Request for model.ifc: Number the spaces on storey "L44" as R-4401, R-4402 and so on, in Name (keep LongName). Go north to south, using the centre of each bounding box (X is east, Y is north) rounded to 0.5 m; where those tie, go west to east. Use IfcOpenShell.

First a look at what the model holds.

```python
import ifcopenshell
import ifcopenshell.util.element
import ifcopenshell.util.placement

model = ifcopenshell.open("model.ifc")
print(model.schema)
storey = next(s for s in model.by_type("IfcBuildingStorey") if s.Name == "L44")
spaces = [e for e in ifcopenshell.util.element.get_decomposition(storey) if e.is_a("IfcSpace")]
for e in sorted(spaces, key=lambda e: e.id()):
    origin = ifcopenshell.util.placement.get_local_placement(e.ObjectPlacement)[:3, 3]
    print(e.id(), e.Name, e.LongName, origin.round(2) + 0.0, sep=" | ")
```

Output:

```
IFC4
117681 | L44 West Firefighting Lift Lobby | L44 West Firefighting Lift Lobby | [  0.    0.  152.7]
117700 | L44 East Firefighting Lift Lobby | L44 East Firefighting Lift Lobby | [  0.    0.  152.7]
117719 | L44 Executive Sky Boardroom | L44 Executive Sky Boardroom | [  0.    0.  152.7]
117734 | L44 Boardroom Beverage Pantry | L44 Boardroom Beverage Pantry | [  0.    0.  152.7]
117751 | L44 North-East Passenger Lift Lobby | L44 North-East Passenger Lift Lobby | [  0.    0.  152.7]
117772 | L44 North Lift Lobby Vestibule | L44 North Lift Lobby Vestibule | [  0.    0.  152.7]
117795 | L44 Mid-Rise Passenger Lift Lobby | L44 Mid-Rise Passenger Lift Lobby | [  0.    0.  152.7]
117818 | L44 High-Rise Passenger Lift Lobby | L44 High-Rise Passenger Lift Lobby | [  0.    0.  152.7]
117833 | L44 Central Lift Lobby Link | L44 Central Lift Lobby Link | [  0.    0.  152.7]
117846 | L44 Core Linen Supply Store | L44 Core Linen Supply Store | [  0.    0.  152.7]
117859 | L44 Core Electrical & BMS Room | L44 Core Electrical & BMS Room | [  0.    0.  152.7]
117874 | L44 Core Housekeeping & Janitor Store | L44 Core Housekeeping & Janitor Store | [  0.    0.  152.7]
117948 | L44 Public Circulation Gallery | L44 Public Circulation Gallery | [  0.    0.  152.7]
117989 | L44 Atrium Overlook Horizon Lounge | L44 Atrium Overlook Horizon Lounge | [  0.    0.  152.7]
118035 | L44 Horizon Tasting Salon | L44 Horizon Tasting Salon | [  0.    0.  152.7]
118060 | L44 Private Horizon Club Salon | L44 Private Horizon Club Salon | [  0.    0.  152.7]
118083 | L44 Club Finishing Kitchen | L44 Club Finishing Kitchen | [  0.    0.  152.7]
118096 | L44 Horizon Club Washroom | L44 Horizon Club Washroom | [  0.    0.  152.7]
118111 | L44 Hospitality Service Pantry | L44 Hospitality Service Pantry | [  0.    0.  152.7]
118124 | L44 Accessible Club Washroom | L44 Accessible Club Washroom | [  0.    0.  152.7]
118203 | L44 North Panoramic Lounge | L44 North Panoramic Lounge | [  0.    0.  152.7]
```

```python
import ifcopenshell
import ifcopenshell.geom
import ifcopenshell.util.element
import ifcopenshell.util.shape

model = ifcopenshell.open("model.ifc")
settings = ifcopenshell.geom.settings()
settings.set("use-world-coords", True)


def centre(element):
    shape = ifcopenshell.geom.create_shape(settings, element)
    return ifcopenshell.util.shape.get_bbox_centroid(shape.geometry)


storey = next(s for s in model.by_type("IfcBuildingStorey") if s.Name == "L44")
spaces = [e for e in ifcopenshell.util.element.get_decomposition(storey) if e.is_a("IfcSpace")]

# Insertion points can sit at a corner or the storey origin, so sort by the geometry (in metres).
centres = {e: centre(e) for e in spaces}
spaces.sort(key=lambda e: (-round(centres[e][1] / 0.5), centres[e][0]))

for i, e in enumerate(spaces, start=1):
    number = f"R-44{i:02d}"
    e.Name = number
    print(e.id(), number)

model.write("model_rev.ifc")
```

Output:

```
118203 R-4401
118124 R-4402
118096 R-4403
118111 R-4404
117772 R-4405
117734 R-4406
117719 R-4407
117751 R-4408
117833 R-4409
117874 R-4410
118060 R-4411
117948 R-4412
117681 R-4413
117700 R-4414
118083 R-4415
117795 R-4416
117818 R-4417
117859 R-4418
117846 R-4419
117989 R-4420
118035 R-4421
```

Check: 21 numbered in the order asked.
